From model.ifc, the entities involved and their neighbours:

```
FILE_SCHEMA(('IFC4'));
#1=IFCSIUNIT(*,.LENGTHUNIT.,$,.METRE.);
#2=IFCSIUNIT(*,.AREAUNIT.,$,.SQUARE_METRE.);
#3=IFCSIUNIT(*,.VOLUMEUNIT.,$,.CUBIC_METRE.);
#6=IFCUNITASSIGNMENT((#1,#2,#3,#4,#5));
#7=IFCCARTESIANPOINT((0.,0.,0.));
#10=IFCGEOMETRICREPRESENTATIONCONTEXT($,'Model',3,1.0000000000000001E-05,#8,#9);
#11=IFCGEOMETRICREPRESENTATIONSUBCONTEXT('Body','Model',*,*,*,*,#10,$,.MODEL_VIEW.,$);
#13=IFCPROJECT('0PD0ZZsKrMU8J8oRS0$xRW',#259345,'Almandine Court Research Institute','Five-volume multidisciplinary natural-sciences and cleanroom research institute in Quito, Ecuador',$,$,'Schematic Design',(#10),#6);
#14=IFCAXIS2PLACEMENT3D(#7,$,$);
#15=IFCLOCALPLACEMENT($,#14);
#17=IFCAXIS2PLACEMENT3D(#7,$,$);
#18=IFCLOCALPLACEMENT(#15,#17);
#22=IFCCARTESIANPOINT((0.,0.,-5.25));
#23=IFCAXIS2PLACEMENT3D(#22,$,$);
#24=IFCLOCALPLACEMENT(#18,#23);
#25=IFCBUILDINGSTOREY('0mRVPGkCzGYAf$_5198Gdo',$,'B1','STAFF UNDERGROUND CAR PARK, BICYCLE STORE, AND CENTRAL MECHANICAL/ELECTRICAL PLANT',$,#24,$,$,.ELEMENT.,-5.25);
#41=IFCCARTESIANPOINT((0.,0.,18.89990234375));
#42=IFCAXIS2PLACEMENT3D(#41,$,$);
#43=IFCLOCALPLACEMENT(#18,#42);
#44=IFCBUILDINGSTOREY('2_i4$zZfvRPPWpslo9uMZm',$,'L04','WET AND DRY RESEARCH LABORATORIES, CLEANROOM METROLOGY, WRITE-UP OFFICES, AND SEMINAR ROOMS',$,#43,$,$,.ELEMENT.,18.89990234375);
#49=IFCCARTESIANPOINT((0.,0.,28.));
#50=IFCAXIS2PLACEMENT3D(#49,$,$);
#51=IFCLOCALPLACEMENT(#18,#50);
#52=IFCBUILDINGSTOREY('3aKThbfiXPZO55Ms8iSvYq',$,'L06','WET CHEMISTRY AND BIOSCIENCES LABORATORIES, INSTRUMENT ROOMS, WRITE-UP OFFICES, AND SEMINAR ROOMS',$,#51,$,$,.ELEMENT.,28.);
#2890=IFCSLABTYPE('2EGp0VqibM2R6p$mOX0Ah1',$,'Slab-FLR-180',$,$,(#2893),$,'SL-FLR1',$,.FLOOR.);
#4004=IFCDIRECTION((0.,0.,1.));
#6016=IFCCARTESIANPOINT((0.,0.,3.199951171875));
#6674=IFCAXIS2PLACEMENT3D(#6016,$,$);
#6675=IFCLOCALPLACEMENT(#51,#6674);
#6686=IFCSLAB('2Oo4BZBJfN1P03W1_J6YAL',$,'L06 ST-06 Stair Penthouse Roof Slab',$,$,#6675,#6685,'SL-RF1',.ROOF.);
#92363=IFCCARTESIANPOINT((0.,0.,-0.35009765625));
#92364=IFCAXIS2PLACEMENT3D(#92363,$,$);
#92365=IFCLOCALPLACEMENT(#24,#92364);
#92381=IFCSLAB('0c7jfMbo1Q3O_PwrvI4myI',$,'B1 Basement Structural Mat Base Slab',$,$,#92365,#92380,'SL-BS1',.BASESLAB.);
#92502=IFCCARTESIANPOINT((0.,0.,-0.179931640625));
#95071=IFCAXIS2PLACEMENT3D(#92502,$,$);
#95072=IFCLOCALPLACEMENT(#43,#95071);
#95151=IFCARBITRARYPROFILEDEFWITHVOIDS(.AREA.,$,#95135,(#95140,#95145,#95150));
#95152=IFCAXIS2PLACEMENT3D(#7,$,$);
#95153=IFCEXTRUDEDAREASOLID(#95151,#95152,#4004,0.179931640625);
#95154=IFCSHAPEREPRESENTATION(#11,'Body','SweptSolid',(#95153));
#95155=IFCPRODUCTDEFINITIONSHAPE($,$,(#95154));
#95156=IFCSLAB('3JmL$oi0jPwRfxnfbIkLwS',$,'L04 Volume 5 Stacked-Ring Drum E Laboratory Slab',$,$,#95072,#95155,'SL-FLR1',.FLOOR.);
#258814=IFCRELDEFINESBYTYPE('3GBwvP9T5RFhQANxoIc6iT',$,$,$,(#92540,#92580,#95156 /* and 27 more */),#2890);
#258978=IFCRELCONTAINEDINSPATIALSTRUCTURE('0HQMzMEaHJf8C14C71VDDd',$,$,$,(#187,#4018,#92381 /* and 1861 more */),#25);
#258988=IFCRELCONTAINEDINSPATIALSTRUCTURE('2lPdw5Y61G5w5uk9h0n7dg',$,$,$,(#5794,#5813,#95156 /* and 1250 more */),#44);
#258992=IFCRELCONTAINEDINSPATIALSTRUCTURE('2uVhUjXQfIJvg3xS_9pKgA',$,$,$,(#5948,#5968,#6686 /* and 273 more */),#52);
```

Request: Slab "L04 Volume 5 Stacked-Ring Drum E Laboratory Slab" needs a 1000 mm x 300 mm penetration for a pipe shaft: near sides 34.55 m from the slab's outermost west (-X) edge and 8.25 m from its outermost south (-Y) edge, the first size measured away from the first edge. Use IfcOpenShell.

```python
import numpy as np
import ifcopenshell
import ifcopenshell.api.feature
import ifcopenshell.api.geometry
import ifcopenshell.api.root
import ifcopenshell.geom
import ifcopenshell.util.placement
import ifcopenshell.util.representation
import ifcopenshell.util.shape
import ifcopenshell.util.unit

model = ifcopenshell.open("model.ifc")
unit_scale = ifcopenshell.util.unit.calculate_unit_scale(model)
settings = ifcopenshell.geom.settings()


def volume(element):
    """Net volume in cubic metres, openings subtracted."""
    shape = ifcopenshell.geom.create_shape(settings, element)
    return ifcopenshell.util.shape.get_volume(shape.geometry)


slab = model.by_guid("3JmL$oi0jPwRfxnfbIkLwS")
before = volume(slab)

# Extent in the slab's own axes, in metres. The edges named are its -X and -Y sides.
slab_shape = ifcopenshell.geom.create_shape(settings, slab)
vertices = ifcopenshell.util.shape.get_vertices(slab_shape.geometry)
x_min, y_min, bottom = vertices.min(axis=0)
top = vertices[:, 2].max()

opening = ifcopenshell.api.root.create_entity(model, ifc_class="IfcOpeningElement", name="Pipe shaft opening", predefined_type="OPENING")
context = ifcopenshell.util.representation.get_context(model, "Model", "Body", "MODEL_VIEW")
width, depth = 1, 0.3
outline = [(0.0, 0.0), (width, 0.0), (width, depth), (0.0, depth), (0.0, 0.0)]
# Overshoot both faces by 50 mm so the cut is clean.
shape = ifcopenshell.api.geometry.add_slab_representation(
    model, context=context, depth=top - bottom + 0.1, polyline=outline
)
ifcopenshell.api.geometry.assign_representation(model, product=opening, representation=shape)

matrix = ifcopenshell.util.placement.get_local_placement(slab.ObjectPlacement)
matrix[:, 3] = matrix @ np.append(np.array([x_min + 34.55, y_min + 8.25, bottom - 0.05]) / unit_scale, 1.0)
ifcopenshell.api.geometry.edit_object_placement(model, product=opening, matrix=matrix, is_si=False)
ifcopenshell.api.feature.add_feature(model, feature=opening, element=slab)

after = volume(slab)

print(f"slab volume {before:.3f} -> {after:.3f} m3")

model.write("model_v2.ifc")
```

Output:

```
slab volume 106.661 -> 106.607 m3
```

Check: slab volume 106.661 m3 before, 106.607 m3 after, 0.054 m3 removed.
